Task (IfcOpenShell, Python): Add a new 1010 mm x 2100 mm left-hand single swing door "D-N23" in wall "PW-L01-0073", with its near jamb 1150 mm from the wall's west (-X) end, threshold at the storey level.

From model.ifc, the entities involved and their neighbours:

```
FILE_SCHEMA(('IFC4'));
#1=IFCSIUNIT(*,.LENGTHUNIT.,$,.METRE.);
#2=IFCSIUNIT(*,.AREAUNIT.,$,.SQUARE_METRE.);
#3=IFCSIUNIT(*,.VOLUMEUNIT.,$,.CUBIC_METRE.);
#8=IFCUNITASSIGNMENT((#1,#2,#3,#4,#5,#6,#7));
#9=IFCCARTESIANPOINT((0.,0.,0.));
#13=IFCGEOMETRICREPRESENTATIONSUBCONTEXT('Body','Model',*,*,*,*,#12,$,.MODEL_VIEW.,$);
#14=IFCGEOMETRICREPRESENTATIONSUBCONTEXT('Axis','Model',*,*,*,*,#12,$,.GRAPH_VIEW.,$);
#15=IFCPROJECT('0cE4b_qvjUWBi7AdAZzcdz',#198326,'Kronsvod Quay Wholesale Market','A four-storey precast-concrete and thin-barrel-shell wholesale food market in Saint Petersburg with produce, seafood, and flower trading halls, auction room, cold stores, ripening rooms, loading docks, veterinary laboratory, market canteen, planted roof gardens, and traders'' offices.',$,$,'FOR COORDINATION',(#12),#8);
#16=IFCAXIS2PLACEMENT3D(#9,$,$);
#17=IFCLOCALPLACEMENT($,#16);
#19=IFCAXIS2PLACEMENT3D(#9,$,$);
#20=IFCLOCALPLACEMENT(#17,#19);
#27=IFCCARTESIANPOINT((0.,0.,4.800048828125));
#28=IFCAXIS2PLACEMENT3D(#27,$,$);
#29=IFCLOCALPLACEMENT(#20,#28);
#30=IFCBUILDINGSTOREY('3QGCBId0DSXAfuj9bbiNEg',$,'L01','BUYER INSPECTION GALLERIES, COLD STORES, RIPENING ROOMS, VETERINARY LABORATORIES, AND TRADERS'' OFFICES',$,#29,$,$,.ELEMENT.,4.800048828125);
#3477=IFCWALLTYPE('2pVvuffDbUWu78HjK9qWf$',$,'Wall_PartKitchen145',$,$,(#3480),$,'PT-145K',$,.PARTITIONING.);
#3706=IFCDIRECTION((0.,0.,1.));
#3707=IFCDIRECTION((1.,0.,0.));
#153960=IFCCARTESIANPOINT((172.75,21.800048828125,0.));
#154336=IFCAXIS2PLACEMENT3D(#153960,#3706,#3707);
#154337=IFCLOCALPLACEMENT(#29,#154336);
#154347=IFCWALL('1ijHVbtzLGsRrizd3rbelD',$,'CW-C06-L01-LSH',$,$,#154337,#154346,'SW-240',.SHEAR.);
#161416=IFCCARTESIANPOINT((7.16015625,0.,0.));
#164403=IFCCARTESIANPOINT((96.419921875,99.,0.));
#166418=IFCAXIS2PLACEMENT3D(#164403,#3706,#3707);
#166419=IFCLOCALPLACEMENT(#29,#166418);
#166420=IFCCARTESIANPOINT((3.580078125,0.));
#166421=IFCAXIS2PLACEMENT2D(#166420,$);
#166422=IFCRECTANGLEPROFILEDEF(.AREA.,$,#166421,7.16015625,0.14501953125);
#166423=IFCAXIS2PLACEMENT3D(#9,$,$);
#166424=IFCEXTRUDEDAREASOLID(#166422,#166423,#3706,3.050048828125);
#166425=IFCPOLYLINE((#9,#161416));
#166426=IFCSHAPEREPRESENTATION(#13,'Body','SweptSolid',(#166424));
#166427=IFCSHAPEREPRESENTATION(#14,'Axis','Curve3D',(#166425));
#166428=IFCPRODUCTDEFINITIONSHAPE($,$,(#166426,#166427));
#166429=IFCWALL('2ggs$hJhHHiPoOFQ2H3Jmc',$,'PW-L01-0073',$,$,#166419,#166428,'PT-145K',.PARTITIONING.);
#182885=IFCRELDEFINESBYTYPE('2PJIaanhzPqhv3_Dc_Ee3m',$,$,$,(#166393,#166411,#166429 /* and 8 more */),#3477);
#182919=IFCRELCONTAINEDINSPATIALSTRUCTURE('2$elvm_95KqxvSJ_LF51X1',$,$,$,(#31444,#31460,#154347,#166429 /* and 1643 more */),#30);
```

```python
import numpy as np
import ifcopenshell
import ifcopenshell.api.feature
import ifcopenshell.api.geometry
import ifcopenshell.api.root
import ifcopenshell.api.spatial
import ifcopenshell.geom
import ifcopenshell.util.element
import ifcopenshell.util.placement
import ifcopenshell.util.representation
import ifcopenshell.util.shape
import ifcopenshell.util.unit

model = ifcopenshell.open("model.ifc")
unit_scale = ifcopenshell.util.unit.calculate_unit_scale(model)
settings = ifcopenshell.geom.settings()


def volume(element):
    """Net volume in cubic metres, openings subtracted."""
    shape = ifcopenshell.geom.create_shape(settings, element)
    return ifcopenshell.util.shape.get_volume(shape.geometry)


wall = model.by_guid("2ggs$hJhHHiPoOFQ2H3Jmc")
storey = ifcopenshell.util.element.get_container(wall, ifc_class="IfcBuildingStorey")
context = ifcopenshell.util.representation.get_context(model, "Model", "Body", "MODEL_VIEW")
before = volume(wall)

width, height, from_end, sill = 1.01, 2.1, 1.15, 0.0  # metres

# The wall runs along its own X axis, and the end named is its -X end.
wall_shape = ifcopenshell.geom.create_shape(settings, wall)
x, y, z = ifcopenshell.util.shape.get_vertices(wall_shape.geometry).T
start = x.min() + from_end
face, thickness = float(y.min()), float(y.max() - y.min())
wall_matrix = ifcopenshell.util.placement.get_local_placement(wall.ObjectPlacement)
level = ifcopenshell.util.placement.get_local_placement(storey.ObjectPlacement)[2, 3]


def in_wall(x, y):
    """Placement at x, y metres in the wall's axes, at sill height."""
    matrix = wall_matrix.copy()
    matrix[:, 3] = wall_matrix @ np.array([x / unit_scale, y / unit_scale, 0.0, 1.0])
    matrix[2, 3] = level + sill / unit_scale
    return matrix


# Opening: a box that overshoots both wall faces by 50 mm.
opening = ifcopenshell.api.root.create_entity(model, ifc_class="IfcOpeningElement", predefined_type="OPENING")
box = ifcopenshell.api.geometry.add_wall_representation(
    model, context=context, length=width, height=height, thickness=thickness + 0.1
)
ifcopenshell.api.geometry.assign_representation(model, product=opening, representation=box)
ifcopenshell.api.geometry.edit_object_placement(model, product=opening, matrix=in_wall(start, face - 0.05), is_si=False)
ifcopenshell.api.feature.add_feature(model, feature=opening, element=wall)

door = ifcopenshell.api.root.create_entity(model, ifc_class="IfcDoor", name="D-N23", predefined_type="DOOR")
door.OverallWidth, door.OverallHeight = width / unit_scale, height / unit_scale
door.OperationType = "SINGLE_SWING_LEFT"
body = ifcopenshell.api.geometry.add_door_representation(
    model,
    context=context,
    overall_width=door.OverallWidth,
    overall_height=door.OverallHeight,
    operation_type="SINGLE_SWING_LEFT",
    lining_properties={"LiningDepth": thickness / unit_scale, "ThresholdDepth": thickness / unit_scale},
)
ifcopenshell.api.geometry.assign_representation(model, product=door, representation=body)
ifcopenshell.api.spatial.assign_container(model, products=[door], relating_structure=storey)
ifcopenshell.api.feature.add_filling(model, opening=opening, element=door)

# The lining spans the wall, so the door starts at the wall face.
ifcopenshell.api.geometry.edit_object_placement(model, product=door, matrix=in_wall(start, face), is_si=False)

after = volume(wall)

print(f"wall volume {before:.3f} -> {after:.3f} m3")

model.write("model_v2.ifc")
```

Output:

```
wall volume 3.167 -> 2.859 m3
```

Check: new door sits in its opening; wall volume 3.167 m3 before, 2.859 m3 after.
